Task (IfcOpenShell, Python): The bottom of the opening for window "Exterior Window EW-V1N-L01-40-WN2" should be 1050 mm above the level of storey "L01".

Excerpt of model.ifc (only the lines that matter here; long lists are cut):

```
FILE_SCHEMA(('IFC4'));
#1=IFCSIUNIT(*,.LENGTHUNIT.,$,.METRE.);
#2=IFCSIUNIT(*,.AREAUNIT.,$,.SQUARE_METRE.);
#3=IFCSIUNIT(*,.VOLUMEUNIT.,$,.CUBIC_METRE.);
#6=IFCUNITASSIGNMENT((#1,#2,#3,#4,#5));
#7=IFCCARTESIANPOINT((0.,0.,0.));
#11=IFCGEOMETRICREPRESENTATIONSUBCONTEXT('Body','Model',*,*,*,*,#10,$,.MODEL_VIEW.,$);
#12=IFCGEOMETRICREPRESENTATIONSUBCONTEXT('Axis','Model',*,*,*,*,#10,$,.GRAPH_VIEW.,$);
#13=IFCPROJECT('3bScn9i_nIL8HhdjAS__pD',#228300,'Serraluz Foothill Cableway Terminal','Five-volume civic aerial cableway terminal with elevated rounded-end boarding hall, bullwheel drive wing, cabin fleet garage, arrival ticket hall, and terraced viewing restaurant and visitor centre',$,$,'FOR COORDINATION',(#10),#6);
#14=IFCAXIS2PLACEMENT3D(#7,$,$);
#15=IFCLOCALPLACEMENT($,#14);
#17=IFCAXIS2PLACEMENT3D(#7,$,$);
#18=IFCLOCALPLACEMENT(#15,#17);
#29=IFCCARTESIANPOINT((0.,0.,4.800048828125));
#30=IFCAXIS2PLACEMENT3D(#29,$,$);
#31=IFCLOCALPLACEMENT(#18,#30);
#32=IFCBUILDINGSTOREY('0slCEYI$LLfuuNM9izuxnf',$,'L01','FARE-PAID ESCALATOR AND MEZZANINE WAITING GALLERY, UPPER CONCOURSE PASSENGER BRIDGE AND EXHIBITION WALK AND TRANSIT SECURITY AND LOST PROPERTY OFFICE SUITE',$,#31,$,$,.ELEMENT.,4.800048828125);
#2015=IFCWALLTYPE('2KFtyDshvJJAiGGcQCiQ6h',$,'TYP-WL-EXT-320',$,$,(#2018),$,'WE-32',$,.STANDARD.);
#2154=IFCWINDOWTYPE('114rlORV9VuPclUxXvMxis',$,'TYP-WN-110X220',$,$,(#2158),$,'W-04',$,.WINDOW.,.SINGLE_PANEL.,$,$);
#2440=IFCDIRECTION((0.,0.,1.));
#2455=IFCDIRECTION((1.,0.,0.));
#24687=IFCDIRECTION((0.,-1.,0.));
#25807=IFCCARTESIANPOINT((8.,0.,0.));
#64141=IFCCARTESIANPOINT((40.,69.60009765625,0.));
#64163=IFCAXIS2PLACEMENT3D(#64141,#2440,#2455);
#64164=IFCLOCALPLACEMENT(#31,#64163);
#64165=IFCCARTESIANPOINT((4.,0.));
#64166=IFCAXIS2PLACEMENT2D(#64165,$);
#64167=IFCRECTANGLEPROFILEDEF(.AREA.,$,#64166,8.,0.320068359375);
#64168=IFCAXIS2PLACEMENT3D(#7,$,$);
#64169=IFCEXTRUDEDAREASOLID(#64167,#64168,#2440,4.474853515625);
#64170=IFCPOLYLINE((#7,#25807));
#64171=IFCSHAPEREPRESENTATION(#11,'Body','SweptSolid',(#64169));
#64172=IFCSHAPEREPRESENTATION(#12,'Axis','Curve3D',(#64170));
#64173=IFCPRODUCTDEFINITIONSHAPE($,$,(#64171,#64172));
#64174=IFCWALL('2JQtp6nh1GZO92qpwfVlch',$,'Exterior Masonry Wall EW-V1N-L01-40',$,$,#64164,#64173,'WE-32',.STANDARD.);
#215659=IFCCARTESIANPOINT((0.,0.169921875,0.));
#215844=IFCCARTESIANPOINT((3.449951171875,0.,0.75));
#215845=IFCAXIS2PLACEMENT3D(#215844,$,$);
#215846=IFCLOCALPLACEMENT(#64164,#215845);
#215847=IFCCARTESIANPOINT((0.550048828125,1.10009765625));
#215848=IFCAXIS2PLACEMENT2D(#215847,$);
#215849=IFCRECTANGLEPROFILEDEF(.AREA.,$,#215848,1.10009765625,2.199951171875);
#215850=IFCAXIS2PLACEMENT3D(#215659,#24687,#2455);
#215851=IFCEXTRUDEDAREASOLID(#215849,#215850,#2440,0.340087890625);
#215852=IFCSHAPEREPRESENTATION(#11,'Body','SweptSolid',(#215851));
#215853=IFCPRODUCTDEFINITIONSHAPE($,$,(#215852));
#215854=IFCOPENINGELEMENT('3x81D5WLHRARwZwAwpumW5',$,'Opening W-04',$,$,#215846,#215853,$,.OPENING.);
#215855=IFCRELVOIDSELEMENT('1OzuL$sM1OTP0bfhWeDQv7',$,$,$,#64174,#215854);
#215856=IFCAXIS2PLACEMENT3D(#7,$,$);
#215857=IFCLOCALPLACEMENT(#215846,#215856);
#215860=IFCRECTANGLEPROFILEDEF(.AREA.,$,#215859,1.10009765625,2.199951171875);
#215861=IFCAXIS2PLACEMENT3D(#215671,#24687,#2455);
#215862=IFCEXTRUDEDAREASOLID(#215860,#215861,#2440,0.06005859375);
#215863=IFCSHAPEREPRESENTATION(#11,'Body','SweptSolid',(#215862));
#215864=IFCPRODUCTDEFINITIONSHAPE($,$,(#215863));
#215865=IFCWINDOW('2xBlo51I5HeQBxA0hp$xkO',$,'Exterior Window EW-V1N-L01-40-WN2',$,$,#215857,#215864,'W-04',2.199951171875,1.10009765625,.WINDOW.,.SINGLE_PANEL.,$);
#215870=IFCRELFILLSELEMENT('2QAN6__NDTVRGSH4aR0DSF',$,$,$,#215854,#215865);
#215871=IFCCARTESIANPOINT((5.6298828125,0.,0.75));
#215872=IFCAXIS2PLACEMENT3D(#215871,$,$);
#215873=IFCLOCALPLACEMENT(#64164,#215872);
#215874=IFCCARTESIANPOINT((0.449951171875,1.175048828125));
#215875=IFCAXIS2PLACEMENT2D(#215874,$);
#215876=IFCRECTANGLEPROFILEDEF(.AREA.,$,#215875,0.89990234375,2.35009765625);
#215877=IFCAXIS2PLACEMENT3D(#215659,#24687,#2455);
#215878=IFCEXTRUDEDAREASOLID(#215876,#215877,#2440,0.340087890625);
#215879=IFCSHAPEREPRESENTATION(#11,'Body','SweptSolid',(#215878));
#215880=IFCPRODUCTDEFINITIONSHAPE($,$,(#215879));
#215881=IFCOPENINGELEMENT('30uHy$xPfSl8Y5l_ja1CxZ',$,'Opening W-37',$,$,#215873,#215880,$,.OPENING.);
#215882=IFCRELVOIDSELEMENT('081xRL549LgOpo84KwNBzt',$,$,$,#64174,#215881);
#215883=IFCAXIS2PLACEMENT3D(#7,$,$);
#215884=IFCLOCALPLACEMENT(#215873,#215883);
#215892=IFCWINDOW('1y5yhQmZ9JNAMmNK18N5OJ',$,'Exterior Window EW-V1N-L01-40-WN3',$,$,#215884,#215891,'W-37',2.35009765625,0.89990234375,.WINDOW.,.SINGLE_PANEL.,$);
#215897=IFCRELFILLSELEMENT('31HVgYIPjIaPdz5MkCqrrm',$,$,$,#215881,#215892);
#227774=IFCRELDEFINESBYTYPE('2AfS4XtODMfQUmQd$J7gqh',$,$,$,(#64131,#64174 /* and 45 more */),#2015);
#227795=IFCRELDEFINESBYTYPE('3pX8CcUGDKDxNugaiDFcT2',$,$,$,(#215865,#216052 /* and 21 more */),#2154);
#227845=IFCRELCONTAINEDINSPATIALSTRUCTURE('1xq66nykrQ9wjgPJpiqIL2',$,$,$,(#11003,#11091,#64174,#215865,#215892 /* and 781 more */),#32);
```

```python
import numpy as np
import ifcopenshell
import ifcopenshell.api.geometry
import ifcopenshell.geom
import ifcopenshell.util.element
import ifcopenshell.util.placement
import ifcopenshell.util.shape
import ifcopenshell.util.unit

model = ifcopenshell.open("model.ifc")
unit_scale = ifcopenshell.util.unit.calculate_unit_scale(model)

window = model.by_id(215865)
opening = window.FillsVoids[0].RelatingOpeningElement
storey = ifcopenshell.util.element.get_container(window, ifc_class="IfcBuildingStorey")
level = ifcopenshell.util.placement.get_local_placement(storey.ObjectPlacement)[2, 3]

# The opening's origin need not be at the sill, so measure its lowest point.
shape = ifcopenshell.geom.create_shape(ifcopenshell.geom.settings(), opening)
bottom = ifcopenshell.util.shape.get_shape_bottom_elevation(shape, shape.geometry) / unit_scale
dz = level + 1.05 / unit_scale - bottom

shift = np.array([0.0, 0.0, dz])
# The window is placed relative to its opening, so it follows when the opening moves.
matrix = ifcopenshell.util.placement.get_local_placement(opening.ObjectPlacement)
matrix[:3, 3] += shift
ifcopenshell.api.geometry.edit_object_placement(
    model, product=opening, matrix=matrix, is_si=False, should_transform_children=True
)

print(f"moved by {dz * unit_scale:+.3f} m")

model.write("model_rev.ifc")
```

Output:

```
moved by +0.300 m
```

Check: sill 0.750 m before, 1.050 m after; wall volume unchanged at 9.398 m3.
